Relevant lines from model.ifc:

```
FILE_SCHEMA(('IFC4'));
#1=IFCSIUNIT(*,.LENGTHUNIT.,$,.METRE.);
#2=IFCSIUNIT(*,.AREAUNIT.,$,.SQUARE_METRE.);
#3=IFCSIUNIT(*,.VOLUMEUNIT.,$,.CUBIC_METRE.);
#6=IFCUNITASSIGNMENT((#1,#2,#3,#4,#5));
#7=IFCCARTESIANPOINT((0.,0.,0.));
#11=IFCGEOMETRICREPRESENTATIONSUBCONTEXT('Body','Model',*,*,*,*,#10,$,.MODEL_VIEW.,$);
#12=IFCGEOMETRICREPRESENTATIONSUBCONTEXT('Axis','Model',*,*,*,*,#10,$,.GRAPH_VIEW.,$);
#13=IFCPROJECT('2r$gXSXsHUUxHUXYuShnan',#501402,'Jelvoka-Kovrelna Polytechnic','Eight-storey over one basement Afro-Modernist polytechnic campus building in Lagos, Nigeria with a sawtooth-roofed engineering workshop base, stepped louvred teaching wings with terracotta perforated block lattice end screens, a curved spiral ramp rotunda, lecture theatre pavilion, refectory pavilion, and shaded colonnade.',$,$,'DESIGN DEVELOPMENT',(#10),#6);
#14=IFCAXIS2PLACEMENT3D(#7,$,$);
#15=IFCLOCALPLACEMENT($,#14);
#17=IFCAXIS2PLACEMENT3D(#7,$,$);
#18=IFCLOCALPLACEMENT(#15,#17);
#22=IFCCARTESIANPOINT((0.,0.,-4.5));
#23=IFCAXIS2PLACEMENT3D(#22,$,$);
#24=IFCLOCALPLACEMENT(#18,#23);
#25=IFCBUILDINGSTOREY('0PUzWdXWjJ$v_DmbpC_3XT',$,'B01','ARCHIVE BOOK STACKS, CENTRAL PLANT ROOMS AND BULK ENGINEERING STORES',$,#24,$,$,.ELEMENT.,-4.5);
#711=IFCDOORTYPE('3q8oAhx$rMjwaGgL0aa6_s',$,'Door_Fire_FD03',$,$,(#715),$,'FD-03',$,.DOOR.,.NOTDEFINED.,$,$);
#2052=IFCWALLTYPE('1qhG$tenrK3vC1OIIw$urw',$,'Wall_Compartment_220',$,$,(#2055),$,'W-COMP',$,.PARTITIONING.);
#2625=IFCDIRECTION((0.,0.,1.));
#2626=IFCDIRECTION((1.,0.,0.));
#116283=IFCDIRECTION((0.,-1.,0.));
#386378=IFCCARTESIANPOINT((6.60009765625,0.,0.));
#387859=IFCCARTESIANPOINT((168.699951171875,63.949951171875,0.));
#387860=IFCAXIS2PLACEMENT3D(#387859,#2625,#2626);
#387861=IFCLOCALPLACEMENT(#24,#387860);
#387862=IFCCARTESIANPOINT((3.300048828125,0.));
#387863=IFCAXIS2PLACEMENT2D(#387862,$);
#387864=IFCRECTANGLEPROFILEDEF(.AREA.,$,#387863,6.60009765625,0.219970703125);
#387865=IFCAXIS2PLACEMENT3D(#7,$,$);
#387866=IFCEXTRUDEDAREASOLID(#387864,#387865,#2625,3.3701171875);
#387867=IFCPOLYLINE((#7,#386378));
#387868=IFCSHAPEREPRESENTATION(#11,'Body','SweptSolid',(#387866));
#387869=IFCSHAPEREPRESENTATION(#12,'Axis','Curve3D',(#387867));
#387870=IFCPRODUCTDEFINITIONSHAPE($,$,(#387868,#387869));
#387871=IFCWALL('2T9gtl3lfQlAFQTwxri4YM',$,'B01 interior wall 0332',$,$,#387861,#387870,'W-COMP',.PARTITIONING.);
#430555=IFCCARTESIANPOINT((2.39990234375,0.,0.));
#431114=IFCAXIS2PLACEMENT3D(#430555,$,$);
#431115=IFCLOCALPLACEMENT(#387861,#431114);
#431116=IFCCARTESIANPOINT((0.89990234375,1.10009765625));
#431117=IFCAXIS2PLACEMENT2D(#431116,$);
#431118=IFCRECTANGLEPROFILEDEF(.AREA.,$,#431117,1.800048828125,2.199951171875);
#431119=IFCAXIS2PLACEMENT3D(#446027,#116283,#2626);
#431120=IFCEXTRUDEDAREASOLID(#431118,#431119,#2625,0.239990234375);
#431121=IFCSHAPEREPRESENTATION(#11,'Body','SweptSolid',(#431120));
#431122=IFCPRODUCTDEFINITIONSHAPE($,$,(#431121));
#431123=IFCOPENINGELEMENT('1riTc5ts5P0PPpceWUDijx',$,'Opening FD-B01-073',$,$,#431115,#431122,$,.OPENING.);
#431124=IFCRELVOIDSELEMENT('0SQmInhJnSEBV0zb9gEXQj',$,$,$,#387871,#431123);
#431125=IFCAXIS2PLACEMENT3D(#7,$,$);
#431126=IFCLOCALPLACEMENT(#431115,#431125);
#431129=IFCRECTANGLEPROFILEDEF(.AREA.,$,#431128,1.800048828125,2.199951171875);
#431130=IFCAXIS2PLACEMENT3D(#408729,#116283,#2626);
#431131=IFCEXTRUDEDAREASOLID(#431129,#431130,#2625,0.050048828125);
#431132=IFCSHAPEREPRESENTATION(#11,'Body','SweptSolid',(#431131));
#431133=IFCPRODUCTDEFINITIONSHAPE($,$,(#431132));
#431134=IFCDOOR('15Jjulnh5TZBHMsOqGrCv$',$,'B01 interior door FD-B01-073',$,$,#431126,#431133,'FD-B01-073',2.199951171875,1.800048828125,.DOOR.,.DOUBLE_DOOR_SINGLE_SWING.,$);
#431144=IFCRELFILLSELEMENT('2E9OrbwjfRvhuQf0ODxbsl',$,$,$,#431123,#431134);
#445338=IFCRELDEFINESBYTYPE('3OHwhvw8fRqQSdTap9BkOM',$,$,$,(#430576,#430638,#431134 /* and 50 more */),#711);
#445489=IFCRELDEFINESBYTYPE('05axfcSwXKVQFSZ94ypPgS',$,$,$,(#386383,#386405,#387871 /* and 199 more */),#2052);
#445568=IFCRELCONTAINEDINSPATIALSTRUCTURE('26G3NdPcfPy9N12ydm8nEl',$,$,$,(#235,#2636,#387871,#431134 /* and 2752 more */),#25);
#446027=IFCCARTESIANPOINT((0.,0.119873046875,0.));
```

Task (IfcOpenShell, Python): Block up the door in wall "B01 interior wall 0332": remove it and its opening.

```python
import ifcopenshell
import ifcopenshell.api.feature
import ifcopenshell.api.root
import ifcopenshell.geom
import ifcopenshell.util.shape

model = ifcopenshell.open("model.ifc")
settings = ifcopenshell.geom.settings()


def volume(element):
    """Net volume in cubic metres, openings subtracted."""
    shape = ifcopenshell.geom.create_shape(settings, element)
    return ifcopenshell.util.shape.get_volume(shape.geometry)


door = model.by_id(431134)
opening = door.FillsVoids[0].RelatingOpeningElement
wall = opening.VoidsElements[0].RelatingBuildingElement
before = volume(wall)

ifcopenshell.api.root.remove_product(model, product=door)
ifcopenshell.api.feature.remove_feature(model, feature=opening)

after = volume(wall)

print(f"wall volume {before:.3f} -> {after:.3f} m3")

model.write("model_v2.ifc")
```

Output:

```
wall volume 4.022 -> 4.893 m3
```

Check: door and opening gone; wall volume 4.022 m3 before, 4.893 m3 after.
